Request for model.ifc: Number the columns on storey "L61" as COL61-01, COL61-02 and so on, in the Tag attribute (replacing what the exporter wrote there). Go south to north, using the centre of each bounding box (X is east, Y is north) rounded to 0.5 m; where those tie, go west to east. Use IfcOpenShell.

First a look at what the model holds.

```python
import ifcopenshell
import ifcopenshell.util.element
import ifcopenshell.util.placement

model = ifcopenshell.open("model.ifc")
print(model.schema)
storey = next(s for s in model.by_type("IfcBuildingStorey") if s.Name == "L61")
columns = [e for e in ifcopenshell.util.element.get_decomposition(storey) if e.is_a("IfcColumn")]
for e in sorted(columns, key=lambda e: e.id()):
    origin = ifcopenshell.util.placement.get_local_placement(e.ObjectPlacement)[:3, 3]
    print(e.id(), e.Tag, e.Name, origin.round(2) + 0.0, sep=" | ")
```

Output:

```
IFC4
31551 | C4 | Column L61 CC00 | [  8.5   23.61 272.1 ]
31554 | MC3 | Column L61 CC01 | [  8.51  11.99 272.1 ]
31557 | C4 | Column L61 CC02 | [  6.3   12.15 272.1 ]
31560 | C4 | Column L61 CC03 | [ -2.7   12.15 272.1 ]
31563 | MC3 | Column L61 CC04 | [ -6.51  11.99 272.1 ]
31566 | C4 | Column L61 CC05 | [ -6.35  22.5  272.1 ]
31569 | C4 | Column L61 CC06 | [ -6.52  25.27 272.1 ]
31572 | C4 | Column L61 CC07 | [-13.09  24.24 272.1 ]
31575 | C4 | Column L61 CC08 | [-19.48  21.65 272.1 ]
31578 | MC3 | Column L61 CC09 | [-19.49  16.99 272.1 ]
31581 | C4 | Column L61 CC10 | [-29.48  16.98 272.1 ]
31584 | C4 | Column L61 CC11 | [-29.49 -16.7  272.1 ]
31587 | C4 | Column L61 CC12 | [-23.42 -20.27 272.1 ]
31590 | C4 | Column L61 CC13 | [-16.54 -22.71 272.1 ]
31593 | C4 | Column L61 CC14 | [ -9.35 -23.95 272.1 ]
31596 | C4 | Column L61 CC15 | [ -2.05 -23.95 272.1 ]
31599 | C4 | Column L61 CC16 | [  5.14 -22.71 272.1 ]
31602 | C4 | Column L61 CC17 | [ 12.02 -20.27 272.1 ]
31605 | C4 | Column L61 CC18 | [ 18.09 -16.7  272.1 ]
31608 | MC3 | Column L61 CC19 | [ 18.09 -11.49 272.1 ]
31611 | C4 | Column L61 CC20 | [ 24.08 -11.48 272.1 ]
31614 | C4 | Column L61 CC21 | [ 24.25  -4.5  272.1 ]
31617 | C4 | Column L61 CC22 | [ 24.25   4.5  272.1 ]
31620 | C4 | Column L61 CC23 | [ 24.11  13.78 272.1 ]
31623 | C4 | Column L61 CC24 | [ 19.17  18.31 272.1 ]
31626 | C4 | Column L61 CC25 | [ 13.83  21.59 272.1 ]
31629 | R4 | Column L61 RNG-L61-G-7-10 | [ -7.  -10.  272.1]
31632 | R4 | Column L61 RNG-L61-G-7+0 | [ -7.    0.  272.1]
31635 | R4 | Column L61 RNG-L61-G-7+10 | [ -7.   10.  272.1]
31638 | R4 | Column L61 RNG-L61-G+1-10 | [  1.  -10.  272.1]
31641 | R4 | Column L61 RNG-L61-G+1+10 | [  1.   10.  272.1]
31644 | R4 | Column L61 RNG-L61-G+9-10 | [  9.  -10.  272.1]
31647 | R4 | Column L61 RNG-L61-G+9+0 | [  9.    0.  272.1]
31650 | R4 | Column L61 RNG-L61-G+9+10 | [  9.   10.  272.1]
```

```python
import ifcopenshell
import ifcopenshell.geom
import ifcopenshell.util.element
import ifcopenshell.util.shape

model = ifcopenshell.open("model.ifc")
settings = ifcopenshell.geom.settings()
settings.set("use-world-coords", True)


def centre(element):
    shape = ifcopenshell.geom.create_shape(settings, element)
    return ifcopenshell.util.shape.get_bbox_centroid(shape.geometry)


storey = next(s for s in model.by_type("IfcBuildingStorey") if s.Name == "L61")
columns = [e for e in ifcopenshell.util.element.get_decomposition(storey) if e.is_a("IfcColumn")]

# Insertion points can sit at a corner or the storey origin, so sort by the geometry (in metres).
centres = {e: centre(e) for e in columns}
columns.sort(key=lambda e: (round(centres[e][1] / 0.5), centres[e][0]))

for i, e in enumerate(columns, start=1):
    number = f"COL61-{i:02d}"
    e.Tag = number
    print(e.id(), number)

model.write("model_edited.ifc")
```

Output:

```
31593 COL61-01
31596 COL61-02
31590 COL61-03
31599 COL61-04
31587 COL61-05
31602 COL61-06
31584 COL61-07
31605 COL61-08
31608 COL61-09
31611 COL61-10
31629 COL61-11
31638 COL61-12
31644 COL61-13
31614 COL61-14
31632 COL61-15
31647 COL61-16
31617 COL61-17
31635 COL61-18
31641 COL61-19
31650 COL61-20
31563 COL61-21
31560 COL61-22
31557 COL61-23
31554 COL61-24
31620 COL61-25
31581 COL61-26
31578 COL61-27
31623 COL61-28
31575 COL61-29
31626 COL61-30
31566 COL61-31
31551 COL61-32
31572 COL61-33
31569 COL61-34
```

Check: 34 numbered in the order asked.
